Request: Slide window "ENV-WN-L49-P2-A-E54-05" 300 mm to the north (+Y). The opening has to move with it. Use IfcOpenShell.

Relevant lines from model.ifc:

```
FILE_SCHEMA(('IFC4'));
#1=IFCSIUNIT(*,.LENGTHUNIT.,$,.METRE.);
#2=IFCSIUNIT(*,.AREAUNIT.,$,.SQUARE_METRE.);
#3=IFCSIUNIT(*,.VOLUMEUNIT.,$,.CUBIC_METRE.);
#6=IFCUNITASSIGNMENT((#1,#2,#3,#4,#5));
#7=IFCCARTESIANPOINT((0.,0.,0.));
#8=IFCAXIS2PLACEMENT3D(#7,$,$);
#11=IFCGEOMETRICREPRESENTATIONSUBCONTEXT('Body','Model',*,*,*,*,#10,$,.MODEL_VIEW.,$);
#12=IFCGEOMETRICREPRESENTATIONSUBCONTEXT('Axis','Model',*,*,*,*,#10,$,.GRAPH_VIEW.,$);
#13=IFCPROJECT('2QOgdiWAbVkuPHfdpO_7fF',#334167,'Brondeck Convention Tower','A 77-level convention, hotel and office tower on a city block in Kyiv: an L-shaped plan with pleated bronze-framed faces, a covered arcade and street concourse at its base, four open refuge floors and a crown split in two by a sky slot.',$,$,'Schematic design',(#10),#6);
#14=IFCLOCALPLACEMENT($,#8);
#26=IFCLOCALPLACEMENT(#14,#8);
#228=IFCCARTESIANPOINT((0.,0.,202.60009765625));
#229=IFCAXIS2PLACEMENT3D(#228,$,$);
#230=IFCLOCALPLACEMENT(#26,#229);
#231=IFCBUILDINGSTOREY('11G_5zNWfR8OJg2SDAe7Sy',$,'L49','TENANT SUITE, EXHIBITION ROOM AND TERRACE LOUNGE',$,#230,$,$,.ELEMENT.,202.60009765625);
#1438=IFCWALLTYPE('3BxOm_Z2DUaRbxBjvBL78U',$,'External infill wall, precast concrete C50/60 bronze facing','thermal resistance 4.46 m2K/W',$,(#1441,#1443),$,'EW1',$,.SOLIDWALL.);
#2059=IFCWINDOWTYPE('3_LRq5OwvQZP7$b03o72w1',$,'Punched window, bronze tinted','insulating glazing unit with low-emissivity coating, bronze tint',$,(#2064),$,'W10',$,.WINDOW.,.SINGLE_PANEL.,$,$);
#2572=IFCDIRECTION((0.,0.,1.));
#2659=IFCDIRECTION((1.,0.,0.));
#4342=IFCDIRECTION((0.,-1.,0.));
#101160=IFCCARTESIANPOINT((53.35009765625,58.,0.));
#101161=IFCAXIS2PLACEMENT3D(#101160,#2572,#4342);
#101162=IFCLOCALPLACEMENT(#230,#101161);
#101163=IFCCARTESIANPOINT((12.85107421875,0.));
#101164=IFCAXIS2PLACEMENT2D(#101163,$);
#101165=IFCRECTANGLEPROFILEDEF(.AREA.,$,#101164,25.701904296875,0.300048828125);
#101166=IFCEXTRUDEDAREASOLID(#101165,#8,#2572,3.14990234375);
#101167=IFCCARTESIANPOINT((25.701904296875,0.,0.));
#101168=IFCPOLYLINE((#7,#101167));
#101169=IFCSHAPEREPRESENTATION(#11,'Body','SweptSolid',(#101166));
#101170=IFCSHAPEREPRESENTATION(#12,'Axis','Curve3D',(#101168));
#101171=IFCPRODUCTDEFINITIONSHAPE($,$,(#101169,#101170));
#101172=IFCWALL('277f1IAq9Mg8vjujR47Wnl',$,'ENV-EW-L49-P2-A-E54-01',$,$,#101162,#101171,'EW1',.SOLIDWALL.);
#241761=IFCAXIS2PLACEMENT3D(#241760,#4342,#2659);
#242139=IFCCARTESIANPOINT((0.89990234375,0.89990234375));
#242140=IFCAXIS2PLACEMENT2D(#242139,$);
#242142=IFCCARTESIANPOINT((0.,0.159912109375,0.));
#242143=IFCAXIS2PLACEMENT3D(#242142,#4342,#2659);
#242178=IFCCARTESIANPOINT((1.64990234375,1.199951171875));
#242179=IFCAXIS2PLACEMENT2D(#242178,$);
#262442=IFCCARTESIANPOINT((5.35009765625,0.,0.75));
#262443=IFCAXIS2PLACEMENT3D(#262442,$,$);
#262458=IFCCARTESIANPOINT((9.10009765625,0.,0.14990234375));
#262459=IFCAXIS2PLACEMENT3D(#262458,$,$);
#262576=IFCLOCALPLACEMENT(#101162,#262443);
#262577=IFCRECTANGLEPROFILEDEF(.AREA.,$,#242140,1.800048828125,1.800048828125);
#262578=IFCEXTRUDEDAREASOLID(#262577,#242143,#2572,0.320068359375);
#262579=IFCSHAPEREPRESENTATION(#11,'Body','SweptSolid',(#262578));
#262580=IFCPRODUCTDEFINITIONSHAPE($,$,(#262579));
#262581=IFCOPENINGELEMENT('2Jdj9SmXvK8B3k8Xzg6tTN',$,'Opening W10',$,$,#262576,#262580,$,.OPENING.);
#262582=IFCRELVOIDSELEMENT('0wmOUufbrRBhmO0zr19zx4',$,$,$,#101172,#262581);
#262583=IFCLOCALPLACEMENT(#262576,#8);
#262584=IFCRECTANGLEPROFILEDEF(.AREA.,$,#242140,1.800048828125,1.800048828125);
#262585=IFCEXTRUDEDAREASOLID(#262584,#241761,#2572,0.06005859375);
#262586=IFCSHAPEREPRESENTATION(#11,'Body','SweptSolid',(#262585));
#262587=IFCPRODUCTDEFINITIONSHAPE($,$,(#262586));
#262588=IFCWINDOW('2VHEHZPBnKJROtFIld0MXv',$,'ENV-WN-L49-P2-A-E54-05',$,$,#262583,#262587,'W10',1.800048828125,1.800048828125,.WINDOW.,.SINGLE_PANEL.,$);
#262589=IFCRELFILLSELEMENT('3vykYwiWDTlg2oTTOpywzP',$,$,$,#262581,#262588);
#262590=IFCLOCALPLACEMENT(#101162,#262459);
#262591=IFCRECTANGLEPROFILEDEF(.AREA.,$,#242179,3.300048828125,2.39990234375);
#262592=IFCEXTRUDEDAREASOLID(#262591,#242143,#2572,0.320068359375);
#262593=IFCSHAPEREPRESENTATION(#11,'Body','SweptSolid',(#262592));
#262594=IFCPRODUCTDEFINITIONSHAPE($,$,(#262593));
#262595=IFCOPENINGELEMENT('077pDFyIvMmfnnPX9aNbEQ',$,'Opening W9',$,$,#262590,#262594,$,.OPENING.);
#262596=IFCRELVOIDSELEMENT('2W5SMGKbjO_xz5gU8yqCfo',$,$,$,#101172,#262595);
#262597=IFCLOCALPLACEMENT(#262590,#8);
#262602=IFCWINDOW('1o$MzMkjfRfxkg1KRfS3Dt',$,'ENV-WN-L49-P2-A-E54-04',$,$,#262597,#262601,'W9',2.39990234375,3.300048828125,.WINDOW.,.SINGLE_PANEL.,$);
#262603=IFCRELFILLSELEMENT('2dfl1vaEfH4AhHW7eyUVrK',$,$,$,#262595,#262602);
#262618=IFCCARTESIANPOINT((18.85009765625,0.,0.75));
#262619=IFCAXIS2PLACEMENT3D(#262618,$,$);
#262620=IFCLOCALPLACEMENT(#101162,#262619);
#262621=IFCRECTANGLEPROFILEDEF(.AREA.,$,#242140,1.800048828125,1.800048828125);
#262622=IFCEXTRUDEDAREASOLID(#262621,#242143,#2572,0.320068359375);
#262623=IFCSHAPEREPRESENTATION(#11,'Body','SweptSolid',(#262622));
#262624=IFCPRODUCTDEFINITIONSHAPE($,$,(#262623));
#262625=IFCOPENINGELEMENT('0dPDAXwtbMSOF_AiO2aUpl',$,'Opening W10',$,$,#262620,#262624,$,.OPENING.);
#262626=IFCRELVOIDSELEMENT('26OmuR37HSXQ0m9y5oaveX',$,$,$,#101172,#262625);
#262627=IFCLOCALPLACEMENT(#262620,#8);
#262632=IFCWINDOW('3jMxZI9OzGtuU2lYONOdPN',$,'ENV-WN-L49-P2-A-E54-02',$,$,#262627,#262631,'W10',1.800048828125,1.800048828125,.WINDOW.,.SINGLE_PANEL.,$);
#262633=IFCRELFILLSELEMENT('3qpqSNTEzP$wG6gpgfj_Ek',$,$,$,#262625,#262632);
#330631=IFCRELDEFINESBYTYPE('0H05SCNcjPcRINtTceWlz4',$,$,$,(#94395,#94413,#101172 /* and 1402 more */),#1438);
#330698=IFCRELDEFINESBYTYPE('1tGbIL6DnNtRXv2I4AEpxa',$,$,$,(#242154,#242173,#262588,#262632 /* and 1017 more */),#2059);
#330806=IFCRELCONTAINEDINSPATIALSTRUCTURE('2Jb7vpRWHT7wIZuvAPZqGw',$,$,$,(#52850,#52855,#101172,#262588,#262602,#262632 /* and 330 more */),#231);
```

```python
import ifcopenshell
import ifcopenshell.api.geometry
import ifcopenshell.util.placement
import ifcopenshell.util.unit

model = ifcopenshell.open("model.ifc")
unit_scale = ifcopenshell.util.unit.calculate_unit_scale(model)

window = model.by_id(262588)
opening = window.FillsVoids[0].RelatingOpeningElement
wall = opening.VoidsElements[0].RelatingBuildingElement

wall_matrix = ifcopenshell.util.placement.get_local_placement(wall.ObjectPlacement)
shift = wall_matrix[:3, 0] * -0.3 / unit_scale
before = ifcopenshell.util.placement.get_local_placement(window.ObjectPlacement)[:3, 3].copy()

# The window is placed relative to its opening, so it follows when the opening moves.
matrix = ifcopenshell.util.placement.get_local_placement(opening.ObjectPlacement)
matrix[:3, 3] += shift
ifcopenshell.api.geometry.edit_object_placement(
    model, product=opening, matrix=matrix, is_si=False, should_transform_children=True
)

after = ifcopenshell.util.placement.get_local_placement(window.ObjectPlacement)[:3, 3]
print("window moved by", (after - before).round(3) + 0.0)

model.write("model-out.ifc")
```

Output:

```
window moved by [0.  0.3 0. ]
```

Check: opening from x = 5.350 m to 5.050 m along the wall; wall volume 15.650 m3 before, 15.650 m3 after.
